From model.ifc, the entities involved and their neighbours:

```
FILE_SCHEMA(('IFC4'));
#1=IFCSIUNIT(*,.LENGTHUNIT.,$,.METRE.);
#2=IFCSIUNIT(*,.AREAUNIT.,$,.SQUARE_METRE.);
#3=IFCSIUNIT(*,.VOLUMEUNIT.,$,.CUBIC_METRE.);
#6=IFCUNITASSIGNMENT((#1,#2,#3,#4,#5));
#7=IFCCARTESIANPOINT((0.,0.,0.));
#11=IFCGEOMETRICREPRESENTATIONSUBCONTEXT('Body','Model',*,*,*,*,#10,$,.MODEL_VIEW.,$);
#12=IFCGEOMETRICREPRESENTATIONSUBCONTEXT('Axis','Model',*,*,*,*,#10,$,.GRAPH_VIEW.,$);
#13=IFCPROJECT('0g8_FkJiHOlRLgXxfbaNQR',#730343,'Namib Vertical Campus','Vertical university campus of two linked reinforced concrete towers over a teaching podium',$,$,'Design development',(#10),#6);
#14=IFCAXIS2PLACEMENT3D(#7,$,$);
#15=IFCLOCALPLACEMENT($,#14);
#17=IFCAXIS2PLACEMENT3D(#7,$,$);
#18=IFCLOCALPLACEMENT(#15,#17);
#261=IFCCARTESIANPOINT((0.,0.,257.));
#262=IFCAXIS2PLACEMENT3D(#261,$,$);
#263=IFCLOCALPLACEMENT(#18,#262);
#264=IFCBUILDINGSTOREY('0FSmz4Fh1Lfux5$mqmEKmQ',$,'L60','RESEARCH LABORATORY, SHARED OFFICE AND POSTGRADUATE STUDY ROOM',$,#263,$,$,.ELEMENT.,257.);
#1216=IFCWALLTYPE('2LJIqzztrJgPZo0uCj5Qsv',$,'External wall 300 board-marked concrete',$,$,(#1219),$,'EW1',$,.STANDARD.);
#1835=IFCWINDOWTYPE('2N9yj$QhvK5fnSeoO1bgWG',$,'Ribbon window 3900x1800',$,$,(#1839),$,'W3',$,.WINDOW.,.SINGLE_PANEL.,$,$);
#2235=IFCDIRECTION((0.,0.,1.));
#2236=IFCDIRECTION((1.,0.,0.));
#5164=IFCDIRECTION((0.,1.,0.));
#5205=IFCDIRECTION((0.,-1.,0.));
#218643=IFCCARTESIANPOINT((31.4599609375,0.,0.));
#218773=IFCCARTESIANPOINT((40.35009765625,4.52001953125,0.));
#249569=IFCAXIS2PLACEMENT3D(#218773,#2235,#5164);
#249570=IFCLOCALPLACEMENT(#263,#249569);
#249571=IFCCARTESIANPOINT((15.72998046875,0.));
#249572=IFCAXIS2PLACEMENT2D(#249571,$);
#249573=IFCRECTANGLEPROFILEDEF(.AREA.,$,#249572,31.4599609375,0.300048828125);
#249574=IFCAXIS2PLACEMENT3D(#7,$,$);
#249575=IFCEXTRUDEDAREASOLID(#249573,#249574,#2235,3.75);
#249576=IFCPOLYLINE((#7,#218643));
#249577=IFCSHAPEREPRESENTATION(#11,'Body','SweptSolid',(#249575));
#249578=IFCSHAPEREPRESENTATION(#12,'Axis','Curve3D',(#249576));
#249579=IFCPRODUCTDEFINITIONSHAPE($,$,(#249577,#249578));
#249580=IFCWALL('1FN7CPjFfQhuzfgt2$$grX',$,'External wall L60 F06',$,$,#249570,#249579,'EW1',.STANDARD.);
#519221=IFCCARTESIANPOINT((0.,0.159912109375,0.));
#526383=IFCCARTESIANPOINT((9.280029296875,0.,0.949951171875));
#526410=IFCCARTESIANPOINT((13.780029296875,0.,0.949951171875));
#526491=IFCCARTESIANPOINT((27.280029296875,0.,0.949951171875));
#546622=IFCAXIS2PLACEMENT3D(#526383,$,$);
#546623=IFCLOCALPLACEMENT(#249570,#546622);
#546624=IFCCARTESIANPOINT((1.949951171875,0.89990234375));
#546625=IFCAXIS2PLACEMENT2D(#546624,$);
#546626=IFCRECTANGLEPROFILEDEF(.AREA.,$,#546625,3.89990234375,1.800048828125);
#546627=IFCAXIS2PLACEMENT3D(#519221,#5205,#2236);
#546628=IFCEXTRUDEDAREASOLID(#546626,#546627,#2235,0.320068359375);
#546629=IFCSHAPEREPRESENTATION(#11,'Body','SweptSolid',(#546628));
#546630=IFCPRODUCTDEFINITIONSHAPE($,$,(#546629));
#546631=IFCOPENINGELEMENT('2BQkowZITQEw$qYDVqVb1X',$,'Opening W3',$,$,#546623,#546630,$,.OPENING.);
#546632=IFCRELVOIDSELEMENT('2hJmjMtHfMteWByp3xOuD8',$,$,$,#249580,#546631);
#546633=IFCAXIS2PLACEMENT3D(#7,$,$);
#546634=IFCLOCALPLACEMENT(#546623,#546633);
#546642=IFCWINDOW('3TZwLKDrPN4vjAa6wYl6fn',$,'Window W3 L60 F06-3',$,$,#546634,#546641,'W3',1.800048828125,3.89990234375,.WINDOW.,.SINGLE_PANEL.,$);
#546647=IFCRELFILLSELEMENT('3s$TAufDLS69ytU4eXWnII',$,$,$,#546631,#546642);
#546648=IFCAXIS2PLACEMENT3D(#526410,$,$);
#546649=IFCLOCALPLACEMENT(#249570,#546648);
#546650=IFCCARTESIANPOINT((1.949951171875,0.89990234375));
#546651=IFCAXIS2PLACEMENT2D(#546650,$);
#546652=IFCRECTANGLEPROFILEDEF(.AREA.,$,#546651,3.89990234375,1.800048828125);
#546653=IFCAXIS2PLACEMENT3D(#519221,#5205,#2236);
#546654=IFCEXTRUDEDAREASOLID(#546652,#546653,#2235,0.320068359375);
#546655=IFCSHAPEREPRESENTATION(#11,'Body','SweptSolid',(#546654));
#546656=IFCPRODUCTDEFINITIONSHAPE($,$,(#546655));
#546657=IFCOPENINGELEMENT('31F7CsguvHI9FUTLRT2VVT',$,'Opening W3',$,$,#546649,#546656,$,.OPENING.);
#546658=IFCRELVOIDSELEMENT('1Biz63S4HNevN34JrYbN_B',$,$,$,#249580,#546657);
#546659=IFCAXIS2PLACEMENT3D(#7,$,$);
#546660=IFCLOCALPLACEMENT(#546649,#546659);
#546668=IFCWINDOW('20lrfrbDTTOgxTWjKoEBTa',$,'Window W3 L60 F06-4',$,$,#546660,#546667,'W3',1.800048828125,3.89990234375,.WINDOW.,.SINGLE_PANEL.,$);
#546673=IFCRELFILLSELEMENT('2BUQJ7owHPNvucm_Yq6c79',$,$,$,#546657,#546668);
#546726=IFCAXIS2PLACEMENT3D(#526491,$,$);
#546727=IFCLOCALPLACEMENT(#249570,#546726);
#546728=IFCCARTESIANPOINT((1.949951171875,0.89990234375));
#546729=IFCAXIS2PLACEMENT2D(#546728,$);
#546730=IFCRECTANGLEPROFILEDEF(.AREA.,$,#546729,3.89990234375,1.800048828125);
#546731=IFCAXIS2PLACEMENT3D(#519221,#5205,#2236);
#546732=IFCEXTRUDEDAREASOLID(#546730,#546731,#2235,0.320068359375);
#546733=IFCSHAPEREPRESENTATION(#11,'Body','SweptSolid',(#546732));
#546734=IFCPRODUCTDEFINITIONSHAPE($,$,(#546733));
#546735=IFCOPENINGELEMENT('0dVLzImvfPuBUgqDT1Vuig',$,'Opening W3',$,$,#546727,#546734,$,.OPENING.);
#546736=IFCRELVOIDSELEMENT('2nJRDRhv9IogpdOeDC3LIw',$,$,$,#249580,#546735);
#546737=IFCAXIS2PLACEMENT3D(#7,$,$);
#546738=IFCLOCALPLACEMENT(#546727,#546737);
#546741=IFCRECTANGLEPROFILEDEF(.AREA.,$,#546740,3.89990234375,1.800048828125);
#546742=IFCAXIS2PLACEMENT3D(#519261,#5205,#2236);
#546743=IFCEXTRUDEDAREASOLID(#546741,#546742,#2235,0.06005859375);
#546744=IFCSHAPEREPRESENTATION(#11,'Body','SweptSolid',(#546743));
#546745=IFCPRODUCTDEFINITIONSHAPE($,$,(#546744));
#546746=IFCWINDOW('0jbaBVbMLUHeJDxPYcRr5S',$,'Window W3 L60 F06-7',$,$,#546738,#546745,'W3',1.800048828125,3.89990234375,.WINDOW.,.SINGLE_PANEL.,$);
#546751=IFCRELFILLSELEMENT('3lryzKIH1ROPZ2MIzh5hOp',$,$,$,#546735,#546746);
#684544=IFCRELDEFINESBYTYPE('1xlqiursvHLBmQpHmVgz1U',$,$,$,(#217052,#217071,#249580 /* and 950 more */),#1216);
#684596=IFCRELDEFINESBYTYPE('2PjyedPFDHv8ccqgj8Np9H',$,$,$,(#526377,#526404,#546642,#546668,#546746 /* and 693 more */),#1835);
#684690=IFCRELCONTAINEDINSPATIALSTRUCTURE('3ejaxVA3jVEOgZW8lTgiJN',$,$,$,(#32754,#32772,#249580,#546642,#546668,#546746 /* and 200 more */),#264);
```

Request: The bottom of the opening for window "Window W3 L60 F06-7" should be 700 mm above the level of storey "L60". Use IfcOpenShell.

```python
import numpy as np
import ifcopenshell
import ifcopenshell.api.geometry
import ifcopenshell.geom
import ifcopenshell.util.element
import ifcopenshell.util.placement
import ifcopenshell.util.shape
import ifcopenshell.util.unit

model = ifcopenshell.open("model.ifc")
unit_scale = ifcopenshell.util.unit.calculate_unit_scale(model)

window = model.by_guid("0jbaBVbMLUHeJDxPYcRr5S")
opening = window.FillsVoids[0].RelatingOpeningElement
storey = ifcopenshell.util.element.get_container(window, ifc_class="IfcBuildingStorey")
level = ifcopenshell.util.placement.get_local_placement(storey.ObjectPlacement)[2, 3]

# The opening's origin need not be at the sill, so measure its lowest point.
shape = ifcopenshell.geom.create_shape(ifcopenshell.geom.settings(), opening)
bottom = ifcopenshell.util.shape.get_shape_bottom_elevation(shape, shape.geometry) / unit_scale
dz = level + 0.7 / unit_scale - bottom

shift = np.array([0.0, 0.0, dz])
# The window is placed relative to its opening, so it follows when the opening moves.
matrix = ifcopenshell.util.placement.get_local_placement(opening.ObjectPlacement)
matrix[:3, 3] += shift
ifcopenshell.api.geometry.edit_object_placement(
    model, product=opening, matrix=matrix, is_si=False, should_transform_children=True
)

print(f"moved by {dz * unit_scale:+.3f} m")

model.write("model_v2.ifc")
```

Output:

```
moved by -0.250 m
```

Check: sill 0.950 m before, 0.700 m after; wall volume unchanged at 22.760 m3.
